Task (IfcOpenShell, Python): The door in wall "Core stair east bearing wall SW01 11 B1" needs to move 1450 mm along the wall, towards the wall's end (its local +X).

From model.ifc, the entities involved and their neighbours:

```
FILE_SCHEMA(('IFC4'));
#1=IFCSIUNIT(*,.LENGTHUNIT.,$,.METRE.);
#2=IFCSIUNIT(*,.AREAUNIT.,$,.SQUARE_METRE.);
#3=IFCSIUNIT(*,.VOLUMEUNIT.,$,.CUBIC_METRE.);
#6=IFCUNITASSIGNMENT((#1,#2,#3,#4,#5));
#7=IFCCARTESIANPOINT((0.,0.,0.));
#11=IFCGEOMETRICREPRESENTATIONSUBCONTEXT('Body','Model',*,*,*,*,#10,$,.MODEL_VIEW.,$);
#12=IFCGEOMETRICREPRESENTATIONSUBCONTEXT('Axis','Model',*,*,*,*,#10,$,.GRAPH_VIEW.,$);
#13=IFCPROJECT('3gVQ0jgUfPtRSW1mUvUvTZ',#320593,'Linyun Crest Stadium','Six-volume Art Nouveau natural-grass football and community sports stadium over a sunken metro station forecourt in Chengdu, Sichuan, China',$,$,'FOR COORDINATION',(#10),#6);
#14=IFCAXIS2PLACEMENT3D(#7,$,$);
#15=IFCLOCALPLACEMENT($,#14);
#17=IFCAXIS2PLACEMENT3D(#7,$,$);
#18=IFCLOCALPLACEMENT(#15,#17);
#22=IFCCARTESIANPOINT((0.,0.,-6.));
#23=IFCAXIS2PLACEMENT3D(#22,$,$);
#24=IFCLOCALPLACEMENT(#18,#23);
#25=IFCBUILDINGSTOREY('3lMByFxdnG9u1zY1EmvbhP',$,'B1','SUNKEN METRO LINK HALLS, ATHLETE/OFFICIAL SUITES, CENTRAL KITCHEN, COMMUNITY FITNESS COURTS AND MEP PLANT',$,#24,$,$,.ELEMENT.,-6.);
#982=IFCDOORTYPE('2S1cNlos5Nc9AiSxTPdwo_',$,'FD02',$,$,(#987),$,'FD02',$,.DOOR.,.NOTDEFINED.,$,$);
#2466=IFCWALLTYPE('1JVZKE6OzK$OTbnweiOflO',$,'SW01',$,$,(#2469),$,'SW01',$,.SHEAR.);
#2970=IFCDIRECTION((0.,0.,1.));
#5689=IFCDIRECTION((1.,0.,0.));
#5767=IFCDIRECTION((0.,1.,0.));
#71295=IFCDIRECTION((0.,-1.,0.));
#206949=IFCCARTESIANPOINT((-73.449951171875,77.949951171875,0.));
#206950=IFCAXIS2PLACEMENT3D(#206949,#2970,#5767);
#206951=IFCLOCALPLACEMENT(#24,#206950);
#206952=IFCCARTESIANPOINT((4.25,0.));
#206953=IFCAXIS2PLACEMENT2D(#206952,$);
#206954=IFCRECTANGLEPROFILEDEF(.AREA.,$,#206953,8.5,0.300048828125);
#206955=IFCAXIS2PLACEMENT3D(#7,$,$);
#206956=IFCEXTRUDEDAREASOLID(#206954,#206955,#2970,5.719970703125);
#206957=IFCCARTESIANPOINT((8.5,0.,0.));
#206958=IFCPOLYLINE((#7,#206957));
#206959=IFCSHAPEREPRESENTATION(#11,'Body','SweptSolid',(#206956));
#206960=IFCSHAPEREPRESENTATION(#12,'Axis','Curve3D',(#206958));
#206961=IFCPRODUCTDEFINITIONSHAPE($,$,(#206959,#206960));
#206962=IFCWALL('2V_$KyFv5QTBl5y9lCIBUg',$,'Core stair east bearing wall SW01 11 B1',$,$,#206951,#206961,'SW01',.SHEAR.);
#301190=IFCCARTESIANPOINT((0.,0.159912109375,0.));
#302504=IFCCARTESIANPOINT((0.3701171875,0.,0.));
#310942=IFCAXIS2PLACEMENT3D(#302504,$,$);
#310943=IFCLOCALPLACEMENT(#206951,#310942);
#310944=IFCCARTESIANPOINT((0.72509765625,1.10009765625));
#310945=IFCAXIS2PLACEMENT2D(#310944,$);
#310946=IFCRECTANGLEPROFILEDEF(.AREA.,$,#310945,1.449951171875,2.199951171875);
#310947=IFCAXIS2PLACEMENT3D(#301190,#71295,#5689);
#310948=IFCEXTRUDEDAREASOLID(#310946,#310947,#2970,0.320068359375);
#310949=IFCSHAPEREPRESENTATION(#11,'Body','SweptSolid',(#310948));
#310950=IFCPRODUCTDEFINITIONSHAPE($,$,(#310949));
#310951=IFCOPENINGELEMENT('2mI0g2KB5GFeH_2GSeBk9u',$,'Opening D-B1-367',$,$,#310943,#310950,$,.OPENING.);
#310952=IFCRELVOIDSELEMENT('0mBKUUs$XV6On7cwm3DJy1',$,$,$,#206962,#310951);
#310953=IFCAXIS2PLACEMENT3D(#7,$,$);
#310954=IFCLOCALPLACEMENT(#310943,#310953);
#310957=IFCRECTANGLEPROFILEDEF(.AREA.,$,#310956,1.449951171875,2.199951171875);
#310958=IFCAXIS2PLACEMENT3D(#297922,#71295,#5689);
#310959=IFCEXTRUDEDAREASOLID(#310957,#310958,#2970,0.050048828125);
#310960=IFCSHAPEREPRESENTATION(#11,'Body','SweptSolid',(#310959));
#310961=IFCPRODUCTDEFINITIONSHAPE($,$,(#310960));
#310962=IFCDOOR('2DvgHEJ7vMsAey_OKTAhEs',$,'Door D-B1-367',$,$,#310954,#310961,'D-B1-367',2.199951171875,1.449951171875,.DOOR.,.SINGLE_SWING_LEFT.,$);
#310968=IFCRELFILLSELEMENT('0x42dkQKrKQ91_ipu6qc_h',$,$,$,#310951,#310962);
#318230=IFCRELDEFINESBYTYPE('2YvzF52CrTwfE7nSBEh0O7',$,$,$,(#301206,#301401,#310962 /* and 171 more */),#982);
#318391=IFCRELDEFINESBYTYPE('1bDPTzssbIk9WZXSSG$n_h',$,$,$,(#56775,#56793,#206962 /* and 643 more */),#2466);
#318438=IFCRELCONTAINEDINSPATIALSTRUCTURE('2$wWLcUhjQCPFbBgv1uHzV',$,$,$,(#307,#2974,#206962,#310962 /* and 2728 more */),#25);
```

```python
import ifcopenshell
import ifcopenshell.api.geometry
import ifcopenshell.util.placement
import ifcopenshell.util.unit

model = ifcopenshell.open("model.ifc")
unit_scale = ifcopenshell.util.unit.calculate_unit_scale(model)

door = model.by_id(310962)
opening = door.FillsVoids[0].RelatingOpeningElement
wall = opening.VoidsElements[0].RelatingBuildingElement

wall_matrix = ifcopenshell.util.placement.get_local_placement(wall.ObjectPlacement)
shift = wall_matrix[:3, 0] * 1.45 / unit_scale
before = ifcopenshell.util.placement.get_local_placement(door.ObjectPlacement)[:3, 3].copy()

# The door is placed relative to its opening, so it follows when the opening moves.
matrix = ifcopenshell.util.placement.get_local_placement(opening.ObjectPlacement)
matrix[:3, 3] += shift
ifcopenshell.api.geometry.edit_object_placement(
    model, product=opening, matrix=matrix, is_si=False, should_transform_children=True
)

after = ifcopenshell.util.placement.get_local_placement(door.ObjectPlacement)[:3, 3]
print("door moved by", (after - before).round(3) + 0.0)

model.write("model-out.ifc")
```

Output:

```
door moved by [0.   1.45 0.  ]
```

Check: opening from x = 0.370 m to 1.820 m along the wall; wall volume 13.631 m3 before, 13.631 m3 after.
